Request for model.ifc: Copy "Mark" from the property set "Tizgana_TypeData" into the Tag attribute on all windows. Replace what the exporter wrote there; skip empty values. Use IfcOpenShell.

First a look at what the model holds.

```python
import ifcopenshell
import ifcopenshell.util.element

model = ifcopenshell.open("model.ifc")
print(model.schema)
windows = model.by_type("IfcWindow")
print(len(windows), "windows")
for e in windows[:8]:
    source = ifcopenshell.util.element.get_pset(e, "Tizgana_TypeData", "Mark")
    target = e.Tag
    print(e.id(), repr(source), repr(target), sep=" | ")
```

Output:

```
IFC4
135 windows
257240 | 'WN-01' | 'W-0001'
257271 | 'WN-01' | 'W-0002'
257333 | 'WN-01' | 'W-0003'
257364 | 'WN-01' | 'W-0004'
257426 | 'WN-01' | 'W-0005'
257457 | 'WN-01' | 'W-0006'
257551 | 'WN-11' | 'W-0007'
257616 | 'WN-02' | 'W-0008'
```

```python
import ifcopenshell
import ifcopenshell.util.element

model = ifcopenshell.open("model.ifc")

count = 0
for e in model.by_type("IfcWindow"):
    value = ifcopenshell.util.element.get_pset(e, "Tizgana_TypeData", "Mark")
    current = e.Tag
    if not value or not value.strip() or current == value:
        continue
    e.Tag = value
    count += 1

print(count, "windows updated")

model.write("model_updated.ifc")
```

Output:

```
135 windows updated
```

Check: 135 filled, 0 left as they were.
